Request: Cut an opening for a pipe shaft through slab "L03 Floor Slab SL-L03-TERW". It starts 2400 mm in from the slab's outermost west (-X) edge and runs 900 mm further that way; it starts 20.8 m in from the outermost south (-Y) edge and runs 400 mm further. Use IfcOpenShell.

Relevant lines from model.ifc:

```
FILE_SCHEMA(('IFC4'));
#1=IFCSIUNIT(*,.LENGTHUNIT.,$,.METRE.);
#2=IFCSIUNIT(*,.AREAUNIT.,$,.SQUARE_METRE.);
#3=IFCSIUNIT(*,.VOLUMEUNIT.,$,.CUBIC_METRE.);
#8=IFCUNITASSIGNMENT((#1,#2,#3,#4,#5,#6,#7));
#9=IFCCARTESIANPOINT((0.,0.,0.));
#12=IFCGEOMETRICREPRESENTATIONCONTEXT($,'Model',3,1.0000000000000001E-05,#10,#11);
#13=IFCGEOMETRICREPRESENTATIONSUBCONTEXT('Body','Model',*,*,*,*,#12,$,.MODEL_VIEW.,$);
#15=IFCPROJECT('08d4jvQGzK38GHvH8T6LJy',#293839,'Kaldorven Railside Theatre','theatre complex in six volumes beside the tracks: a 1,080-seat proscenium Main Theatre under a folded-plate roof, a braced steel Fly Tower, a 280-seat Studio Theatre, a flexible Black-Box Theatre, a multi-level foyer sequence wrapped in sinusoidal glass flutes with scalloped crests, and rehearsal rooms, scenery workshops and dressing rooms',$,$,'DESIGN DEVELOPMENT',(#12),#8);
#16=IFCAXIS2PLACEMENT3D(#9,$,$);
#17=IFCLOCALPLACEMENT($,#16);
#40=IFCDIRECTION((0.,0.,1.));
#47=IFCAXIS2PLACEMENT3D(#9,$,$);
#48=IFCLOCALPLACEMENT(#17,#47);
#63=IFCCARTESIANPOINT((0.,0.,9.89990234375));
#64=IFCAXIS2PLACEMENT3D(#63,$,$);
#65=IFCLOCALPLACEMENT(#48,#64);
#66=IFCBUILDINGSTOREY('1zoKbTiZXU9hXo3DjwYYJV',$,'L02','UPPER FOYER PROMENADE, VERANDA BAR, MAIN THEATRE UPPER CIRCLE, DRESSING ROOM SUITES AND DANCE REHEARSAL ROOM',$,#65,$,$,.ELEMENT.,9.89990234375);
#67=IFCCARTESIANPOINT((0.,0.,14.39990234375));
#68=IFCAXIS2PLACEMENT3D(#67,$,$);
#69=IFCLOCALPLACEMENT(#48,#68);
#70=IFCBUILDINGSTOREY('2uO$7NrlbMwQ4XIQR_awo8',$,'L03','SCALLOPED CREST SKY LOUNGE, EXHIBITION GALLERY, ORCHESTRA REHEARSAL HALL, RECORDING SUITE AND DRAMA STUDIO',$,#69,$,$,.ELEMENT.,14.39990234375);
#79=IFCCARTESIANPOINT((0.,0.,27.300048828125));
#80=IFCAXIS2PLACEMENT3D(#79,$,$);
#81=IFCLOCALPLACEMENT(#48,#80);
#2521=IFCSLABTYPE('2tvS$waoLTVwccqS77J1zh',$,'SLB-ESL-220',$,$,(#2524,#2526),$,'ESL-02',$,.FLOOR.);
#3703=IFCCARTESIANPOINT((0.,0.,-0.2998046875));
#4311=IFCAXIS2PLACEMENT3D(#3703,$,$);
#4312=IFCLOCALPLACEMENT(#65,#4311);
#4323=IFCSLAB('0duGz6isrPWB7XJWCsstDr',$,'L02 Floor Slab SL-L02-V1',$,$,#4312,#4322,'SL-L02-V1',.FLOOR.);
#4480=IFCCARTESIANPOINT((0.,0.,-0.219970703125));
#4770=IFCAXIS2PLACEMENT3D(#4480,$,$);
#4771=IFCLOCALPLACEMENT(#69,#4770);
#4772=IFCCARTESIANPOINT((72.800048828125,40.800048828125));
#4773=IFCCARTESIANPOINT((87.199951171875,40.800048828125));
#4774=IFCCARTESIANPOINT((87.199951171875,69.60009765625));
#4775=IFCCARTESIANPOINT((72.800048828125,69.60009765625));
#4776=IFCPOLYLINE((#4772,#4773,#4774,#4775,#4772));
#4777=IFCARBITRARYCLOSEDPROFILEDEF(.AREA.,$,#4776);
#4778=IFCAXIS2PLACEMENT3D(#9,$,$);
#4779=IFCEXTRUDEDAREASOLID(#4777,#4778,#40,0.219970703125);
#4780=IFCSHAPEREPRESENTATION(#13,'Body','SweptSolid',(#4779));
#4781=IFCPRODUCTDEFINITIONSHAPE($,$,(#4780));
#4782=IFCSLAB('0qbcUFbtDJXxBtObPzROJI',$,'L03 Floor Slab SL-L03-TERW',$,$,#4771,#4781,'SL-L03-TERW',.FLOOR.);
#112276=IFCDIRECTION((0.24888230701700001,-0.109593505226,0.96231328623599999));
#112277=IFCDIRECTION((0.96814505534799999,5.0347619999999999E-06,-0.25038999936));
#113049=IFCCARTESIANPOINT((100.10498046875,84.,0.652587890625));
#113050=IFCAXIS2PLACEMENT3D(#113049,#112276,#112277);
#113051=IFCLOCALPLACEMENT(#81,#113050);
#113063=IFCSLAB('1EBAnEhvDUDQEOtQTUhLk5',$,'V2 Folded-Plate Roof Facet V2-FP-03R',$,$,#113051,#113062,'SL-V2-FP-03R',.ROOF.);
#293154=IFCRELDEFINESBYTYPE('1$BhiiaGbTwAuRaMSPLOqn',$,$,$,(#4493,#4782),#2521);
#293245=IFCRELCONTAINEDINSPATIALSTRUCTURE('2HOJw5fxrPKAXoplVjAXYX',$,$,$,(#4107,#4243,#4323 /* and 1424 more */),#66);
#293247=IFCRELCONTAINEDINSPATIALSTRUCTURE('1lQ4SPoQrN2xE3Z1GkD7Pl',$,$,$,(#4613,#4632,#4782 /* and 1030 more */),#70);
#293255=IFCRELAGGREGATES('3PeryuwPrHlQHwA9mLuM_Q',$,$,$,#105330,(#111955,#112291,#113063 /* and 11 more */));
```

```python
import numpy as np
import ifcopenshell
import ifcopenshell.api.feature
import ifcopenshell.api.geometry
import ifcopenshell.api.root
import ifcopenshell.geom
import ifcopenshell.util.placement
import ifcopenshell.util.representation
import ifcopenshell.util.shape
import ifcopenshell.util.unit

model = ifcopenshell.open("model.ifc")
unit_scale = ifcopenshell.util.unit.calculate_unit_scale(model)
settings = ifcopenshell.geom.settings()


def volume(element):
    """Net volume in cubic metres, openings subtracted."""
    shape = ifcopenshell.geom.create_shape(settings, element)
    return ifcopenshell.util.shape.get_volume(shape.geometry)


slab = model.by_guid("0qbcUFbtDJXxBtObPzROJI")
before = volume(slab)

# Extent in the slab's own axes, in metres. The edges named are its -X and -Y sides.
slab_shape = ifcopenshell.geom.create_shape(settings, slab)
vertices = ifcopenshell.util.shape.get_vertices(slab_shape.geometry)
x_min, y_min, bottom = vertices.min(axis=0)
top = vertices[:, 2].max()

opening = ifcopenshell.api.root.create_entity(model, ifc_class="IfcOpeningElement", name="Pipe shaft opening", predefined_type="OPENING")
context = ifcopenshell.util.representation.get_context(model, "Model", "Body", "MODEL_VIEW")
width, depth = 0.9, 0.4
outline = [(0.0, 0.0), (width, 0.0), (width, depth), (0.0, depth), (0.0, 0.0)]
# Overshoot both faces by 50 mm so the cut is clean.
shape = ifcopenshell.api.geometry.add_slab_representation(
    model, context=context, depth=top - bottom + 0.1, polyline=outline
)
ifcopenshell.api.geometry.assign_representation(model, product=opening, representation=shape)

matrix = ifcopenshell.util.placement.get_local_placement(slab.ObjectPlacement)
matrix[:, 3] = matrix @ np.append(np.array([x_min + 2.4, y_min + 20.8, bottom - 0.05]) / unit_scale, 1.0)
ifcopenshell.api.geometry.edit_object_placement(model, product=opening, matrix=matrix, is_si=False)
ifcopenshell.api.feature.add_feature(model, feature=opening, element=slab)

after = volume(slab)

print(f"slab volume {before:.3f} -> {after:.3f} m3")

model.write("model-out.ifc")
```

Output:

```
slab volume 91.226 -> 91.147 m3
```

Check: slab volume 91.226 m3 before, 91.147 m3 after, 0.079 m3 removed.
